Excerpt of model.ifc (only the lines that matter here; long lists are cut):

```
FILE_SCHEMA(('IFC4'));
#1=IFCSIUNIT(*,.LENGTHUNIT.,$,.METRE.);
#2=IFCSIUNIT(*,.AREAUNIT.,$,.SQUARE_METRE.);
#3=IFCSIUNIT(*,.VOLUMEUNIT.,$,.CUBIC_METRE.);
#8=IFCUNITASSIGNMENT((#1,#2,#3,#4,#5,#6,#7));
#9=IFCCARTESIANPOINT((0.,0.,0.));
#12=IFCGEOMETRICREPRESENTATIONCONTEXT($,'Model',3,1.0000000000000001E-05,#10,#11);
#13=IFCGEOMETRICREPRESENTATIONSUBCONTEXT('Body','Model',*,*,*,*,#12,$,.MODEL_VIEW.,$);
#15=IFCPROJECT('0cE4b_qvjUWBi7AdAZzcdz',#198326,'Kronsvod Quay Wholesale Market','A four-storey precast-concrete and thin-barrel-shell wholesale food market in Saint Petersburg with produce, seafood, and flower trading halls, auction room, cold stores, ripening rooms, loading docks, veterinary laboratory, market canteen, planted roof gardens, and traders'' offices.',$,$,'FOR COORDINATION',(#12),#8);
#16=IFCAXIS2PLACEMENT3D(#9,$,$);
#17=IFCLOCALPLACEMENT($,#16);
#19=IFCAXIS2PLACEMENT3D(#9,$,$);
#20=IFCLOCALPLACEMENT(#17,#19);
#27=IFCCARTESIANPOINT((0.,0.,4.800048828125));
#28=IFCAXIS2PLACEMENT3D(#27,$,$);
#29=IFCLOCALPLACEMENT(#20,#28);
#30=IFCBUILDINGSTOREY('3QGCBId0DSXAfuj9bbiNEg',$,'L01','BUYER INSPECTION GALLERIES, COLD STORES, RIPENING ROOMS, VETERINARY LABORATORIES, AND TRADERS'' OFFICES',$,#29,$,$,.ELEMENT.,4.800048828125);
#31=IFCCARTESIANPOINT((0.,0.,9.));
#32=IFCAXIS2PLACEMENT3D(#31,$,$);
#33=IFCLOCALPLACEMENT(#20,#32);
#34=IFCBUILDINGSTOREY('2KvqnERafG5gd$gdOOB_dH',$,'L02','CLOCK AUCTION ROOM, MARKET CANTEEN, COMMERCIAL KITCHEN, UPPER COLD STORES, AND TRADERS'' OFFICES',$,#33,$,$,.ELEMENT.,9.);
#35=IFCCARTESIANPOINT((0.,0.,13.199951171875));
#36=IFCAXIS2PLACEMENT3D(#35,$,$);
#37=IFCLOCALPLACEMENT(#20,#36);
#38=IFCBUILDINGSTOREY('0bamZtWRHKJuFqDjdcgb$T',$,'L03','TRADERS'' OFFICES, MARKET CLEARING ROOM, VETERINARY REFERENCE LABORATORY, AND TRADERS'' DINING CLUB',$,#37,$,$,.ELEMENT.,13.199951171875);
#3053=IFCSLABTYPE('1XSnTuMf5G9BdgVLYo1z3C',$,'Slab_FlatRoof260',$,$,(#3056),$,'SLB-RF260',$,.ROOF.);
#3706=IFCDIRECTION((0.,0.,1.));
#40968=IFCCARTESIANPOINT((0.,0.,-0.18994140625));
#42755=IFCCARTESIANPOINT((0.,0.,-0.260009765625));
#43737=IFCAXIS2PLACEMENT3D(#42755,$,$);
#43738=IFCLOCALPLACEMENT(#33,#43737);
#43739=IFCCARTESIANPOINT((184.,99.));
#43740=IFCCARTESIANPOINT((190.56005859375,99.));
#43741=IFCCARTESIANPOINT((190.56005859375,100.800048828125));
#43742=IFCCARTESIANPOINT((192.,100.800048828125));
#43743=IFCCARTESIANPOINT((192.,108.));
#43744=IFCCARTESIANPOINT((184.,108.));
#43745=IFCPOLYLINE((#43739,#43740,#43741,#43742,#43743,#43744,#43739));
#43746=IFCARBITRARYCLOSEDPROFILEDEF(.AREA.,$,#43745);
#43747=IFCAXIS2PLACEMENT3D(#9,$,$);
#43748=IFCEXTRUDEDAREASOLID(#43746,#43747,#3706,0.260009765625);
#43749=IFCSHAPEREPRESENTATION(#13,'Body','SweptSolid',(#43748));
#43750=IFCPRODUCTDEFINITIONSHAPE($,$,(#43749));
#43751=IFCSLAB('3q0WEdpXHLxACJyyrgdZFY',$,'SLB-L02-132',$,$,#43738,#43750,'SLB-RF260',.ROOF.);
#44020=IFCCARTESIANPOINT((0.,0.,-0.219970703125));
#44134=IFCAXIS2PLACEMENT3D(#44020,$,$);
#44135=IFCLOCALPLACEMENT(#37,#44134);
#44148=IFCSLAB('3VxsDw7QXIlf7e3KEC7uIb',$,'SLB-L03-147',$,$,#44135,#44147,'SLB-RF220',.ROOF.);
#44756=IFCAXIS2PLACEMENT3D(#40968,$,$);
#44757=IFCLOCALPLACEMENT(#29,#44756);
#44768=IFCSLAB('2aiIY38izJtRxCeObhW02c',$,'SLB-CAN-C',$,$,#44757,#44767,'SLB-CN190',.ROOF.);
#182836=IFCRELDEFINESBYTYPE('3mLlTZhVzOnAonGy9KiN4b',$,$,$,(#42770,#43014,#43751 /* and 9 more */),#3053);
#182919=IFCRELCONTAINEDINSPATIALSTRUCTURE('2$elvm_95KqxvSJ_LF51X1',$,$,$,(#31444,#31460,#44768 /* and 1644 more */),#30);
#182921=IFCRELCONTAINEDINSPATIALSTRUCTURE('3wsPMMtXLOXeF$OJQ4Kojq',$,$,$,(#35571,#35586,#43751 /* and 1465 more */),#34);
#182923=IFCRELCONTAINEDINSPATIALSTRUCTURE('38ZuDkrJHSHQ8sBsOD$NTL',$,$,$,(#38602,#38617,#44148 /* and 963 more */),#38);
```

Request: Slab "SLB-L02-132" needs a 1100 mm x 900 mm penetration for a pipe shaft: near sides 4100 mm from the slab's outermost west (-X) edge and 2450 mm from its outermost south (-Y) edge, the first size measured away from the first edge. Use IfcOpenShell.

```python
import numpy as np
import ifcopenshell
import ifcopenshell.api.feature
import ifcopenshell.api.geometry
import ifcopenshell.api.root
import ifcopenshell.geom
import ifcopenshell.util.placement
import ifcopenshell.util.representation
import ifcopenshell.util.shape
import ifcopenshell.util.unit

model = ifcopenshell.open("model.ifc")
unit_scale = ifcopenshell.util.unit.calculate_unit_scale(model)
settings = ifcopenshell.geom.settings()


def volume(element):
    """Net volume in cubic metres, openings subtracted."""
    shape = ifcopenshell.geom.create_shape(settings, element)
    return ifcopenshell.util.shape.get_volume(shape.geometry)


slab = model.by_guid("3q0WEdpXHLxACJyyrgdZFY")
before = volume(slab)

# Extent in the slab's own axes, in metres. The edges named are its -X and -Y sides.
slab_shape = ifcopenshell.geom.create_shape(settings, slab)
vertices = ifcopenshell.util.shape.get_vertices(slab_shape.geometry)
x_min, y_min, bottom = vertices.min(axis=0)
top = vertices[:, 2].max()

opening = ifcopenshell.api.root.create_entity(model, ifc_class="IfcOpeningElement", name="Pipe shaft opening", predefined_type="OPENING")
context = ifcopenshell.util.representation.get_context(model, "Model", "Body", "MODEL_VIEW")
width, depth = 1.1, 0.9
outline = [(0.0, 0.0), (width, 0.0), (width, depth), (0.0, depth), (0.0, 0.0)]
# Overshoot both faces by 50 mm so the cut is clean.
shape = ifcopenshell.api.geometry.add_slab_representation(
    model, context=context, depth=top - bottom + 0.1, polyline=outline
)
ifcopenshell.api.geometry.assign_representation(model, product=opening, representation=shape)

matrix = ifcopenshell.util.placement.get_local_placement(slab.ObjectPlacement)
matrix[:, 3] = matrix @ np.append(np.array([x_min + 4.1, y_min + 2.45, bottom - 0.05]) / unit_scale, 1.0)
ifcopenshell.api.geometry.edit_object_placement(model, product=opening, matrix=matrix, is_si=False)
ifcopenshell.api.feature.add_feature(model, feature=opening, element=slab)

after = volume(slab)

print(f"slab volume {before:.3f} -> {after:.3f} m3")

model.write("model_rev.ifc")
```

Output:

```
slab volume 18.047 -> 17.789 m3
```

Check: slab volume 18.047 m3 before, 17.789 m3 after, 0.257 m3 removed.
